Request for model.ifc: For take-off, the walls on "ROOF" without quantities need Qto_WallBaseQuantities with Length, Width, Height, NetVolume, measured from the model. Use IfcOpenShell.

First a look at what the model holds.

```python
import ifcopenshell
import ifcopenshell.util.element
import ifcopenshell.util.unit

model = ifcopenshell.open("model.ifc")
print(model.schema)
for unit_type in ("LENGTHUNIT", "AREAUNIT", "VOLUMEUNIT"):
    print(unit_type, ifcopenshell.util.unit.calculate_unit_scale(model, unit_type))
storey = next(s for s in model.by_type("IfcBuildingStorey") if s.Name == "ROOF")
walls = [e for e in ifcopenshell.util.element.get_decomposition(storey) if e.is_a("IfcWall")]
for e in sorted(walls, key=lambda e: e.id()):
    print(e.id(), e.is_a(), e.Name, list(ifcopenshell.util.element.get_psets(e, qtos_only=True)), sep=" | ")
```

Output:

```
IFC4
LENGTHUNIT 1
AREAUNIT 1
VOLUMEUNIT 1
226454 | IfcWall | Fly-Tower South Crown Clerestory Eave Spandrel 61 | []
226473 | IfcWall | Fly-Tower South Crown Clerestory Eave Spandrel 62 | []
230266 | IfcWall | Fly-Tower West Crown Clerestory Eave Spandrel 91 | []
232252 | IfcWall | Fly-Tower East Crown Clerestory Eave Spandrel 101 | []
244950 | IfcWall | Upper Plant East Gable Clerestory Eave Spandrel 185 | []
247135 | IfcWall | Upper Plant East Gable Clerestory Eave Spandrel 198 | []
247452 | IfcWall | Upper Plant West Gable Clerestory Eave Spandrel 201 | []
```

```python
import ifcopenshell
import ifcopenshell.api.pset
import ifcopenshell.geom
import ifcopenshell.util.element
import ifcopenshell.util.shape
import ifcopenshell.util.unit

model = ifcopenshell.open("model.ifc")
unit_scale = ifcopenshell.util.unit.calculate_unit_scale(model)
volume_scale = ifcopenshell.util.unit.calculate_unit_scale(model, "VOLUMEUNIT")
settings = ifcopenshell.geom.settings()

storey = next(s for s in model.by_type("IfcBuildingStorey") if s.Name == "ROOF")
walls = [e for e in ifcopenshell.util.element.get_decomposition(storey) if e.is_a("IfcWall")]

for e in sorted(walls, key=lambda e: e.id()):
    if ifcopenshell.util.element.get_psets(e, qtos_only=True, should_inherit=False):
        continue
    # Geometry comes back in metres, in the element's own axes.
    shape = ifcopenshell.geom.create_shape(settings, e)
    values = {
        "Length": ifcopenshell.util.shape.get_x(shape.geometry) / unit_scale,
        "Width": ifcopenshell.util.shape.get_y(shape.geometry) / unit_scale,
        "Height": ifcopenshell.util.shape.get_z(shape.geometry) / unit_scale,
        "NetVolume": ifcopenshell.util.shape.get_volume(shape.geometry) / volume_scale,
    }
    qto = ifcopenshell.api.pset.add_qto(model, product=e, name="Qto_WallBaseQuantities")
    ifcopenshell.api.pset.edit_qto(model, qto=qto, properties=values)
    print(e.id(), {k: round(v, 3) for k, v in values.items()})

model.write("model_rev.ifc")
```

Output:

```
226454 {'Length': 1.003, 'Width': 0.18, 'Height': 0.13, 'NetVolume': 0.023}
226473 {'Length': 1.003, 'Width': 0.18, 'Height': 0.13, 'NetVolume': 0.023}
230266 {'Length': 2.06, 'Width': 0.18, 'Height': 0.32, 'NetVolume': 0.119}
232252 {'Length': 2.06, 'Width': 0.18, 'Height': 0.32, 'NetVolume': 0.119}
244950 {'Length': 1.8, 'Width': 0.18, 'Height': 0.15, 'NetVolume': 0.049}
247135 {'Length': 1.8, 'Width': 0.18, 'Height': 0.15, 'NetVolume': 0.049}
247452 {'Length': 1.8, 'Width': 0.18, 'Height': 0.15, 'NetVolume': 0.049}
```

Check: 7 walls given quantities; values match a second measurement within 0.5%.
